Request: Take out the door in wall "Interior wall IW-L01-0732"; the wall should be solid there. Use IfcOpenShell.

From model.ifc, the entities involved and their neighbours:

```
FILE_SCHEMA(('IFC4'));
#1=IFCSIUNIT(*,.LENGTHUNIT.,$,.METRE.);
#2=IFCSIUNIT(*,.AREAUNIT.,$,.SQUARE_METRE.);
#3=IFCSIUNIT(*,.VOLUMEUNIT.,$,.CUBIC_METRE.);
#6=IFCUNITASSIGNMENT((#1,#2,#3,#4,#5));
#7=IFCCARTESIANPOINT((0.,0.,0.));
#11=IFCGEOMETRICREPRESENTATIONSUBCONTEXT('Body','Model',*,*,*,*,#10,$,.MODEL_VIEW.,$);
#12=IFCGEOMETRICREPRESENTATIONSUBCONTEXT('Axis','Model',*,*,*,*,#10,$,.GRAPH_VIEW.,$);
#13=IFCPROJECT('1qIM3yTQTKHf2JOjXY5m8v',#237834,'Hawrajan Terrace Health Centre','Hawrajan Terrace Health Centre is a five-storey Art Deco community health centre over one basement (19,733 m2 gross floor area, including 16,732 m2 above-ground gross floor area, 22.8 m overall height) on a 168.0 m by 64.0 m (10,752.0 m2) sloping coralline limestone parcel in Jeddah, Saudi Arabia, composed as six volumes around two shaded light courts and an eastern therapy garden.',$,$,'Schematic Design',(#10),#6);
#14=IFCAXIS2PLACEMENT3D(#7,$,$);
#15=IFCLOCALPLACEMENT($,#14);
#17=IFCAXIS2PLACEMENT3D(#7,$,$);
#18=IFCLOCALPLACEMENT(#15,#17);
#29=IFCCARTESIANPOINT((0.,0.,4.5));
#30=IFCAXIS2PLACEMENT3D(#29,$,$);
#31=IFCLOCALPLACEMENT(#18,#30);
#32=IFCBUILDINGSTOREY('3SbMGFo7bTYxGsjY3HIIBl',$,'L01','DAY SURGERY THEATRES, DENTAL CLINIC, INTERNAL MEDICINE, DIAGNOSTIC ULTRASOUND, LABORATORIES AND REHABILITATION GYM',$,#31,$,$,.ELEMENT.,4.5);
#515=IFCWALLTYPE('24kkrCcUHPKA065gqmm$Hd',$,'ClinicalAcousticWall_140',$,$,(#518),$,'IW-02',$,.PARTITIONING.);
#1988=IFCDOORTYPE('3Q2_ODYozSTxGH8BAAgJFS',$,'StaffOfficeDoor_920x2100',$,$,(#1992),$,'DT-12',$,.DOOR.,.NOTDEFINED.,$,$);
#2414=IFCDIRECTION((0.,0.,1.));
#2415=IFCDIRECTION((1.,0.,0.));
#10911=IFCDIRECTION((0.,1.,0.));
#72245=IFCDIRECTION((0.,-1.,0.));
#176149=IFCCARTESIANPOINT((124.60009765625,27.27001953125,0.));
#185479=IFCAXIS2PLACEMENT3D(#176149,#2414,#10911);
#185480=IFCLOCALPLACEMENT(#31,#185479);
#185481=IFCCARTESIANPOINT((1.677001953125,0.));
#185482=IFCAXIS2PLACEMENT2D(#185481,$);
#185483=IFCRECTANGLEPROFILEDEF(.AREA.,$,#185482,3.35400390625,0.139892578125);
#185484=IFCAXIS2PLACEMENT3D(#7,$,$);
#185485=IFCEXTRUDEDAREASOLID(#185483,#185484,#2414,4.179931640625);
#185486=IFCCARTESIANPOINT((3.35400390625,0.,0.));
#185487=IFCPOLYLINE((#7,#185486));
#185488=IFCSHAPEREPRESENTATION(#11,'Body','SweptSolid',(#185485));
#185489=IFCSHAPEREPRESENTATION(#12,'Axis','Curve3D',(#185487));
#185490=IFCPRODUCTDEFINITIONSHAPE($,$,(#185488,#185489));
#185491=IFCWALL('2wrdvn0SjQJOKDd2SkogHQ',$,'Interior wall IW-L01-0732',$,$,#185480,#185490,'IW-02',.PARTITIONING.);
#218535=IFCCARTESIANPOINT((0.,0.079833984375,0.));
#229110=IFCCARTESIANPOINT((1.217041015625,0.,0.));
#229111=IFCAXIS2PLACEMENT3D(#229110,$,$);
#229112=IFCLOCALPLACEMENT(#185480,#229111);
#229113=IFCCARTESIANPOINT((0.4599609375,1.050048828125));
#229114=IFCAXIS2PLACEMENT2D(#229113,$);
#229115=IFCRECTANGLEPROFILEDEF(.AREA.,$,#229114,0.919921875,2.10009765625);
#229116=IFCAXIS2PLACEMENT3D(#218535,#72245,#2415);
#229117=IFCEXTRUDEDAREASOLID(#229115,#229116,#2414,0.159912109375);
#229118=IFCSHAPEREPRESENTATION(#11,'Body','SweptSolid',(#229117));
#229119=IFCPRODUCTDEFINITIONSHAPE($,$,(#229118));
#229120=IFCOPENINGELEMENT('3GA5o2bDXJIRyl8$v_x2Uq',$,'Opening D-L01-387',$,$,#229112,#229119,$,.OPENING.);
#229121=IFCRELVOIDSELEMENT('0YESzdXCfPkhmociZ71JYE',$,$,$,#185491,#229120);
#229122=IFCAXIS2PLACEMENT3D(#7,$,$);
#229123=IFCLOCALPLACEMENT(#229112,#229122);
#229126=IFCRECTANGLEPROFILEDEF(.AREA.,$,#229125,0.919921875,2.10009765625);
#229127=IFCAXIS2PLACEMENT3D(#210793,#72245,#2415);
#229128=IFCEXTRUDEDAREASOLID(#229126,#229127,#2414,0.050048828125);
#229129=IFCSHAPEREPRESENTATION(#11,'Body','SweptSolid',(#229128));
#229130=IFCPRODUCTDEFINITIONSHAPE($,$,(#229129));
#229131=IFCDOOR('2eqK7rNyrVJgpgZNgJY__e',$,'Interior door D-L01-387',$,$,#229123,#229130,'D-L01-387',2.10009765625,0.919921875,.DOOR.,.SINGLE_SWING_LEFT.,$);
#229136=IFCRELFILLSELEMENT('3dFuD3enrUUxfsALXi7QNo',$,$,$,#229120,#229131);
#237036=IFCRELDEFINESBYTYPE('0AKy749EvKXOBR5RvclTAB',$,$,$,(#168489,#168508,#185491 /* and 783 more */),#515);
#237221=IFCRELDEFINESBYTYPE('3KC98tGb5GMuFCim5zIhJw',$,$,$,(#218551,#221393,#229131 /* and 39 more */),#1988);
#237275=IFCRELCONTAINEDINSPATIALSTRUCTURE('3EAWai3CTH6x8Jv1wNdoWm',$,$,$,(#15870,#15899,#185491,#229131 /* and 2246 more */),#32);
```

```python
import ifcopenshell
import ifcopenshell.api.feature
import ifcopenshell.api.root
import ifcopenshell.geom
import ifcopenshell.util.shape

model = ifcopenshell.open("model.ifc")
settings = ifcopenshell.geom.settings()


def volume(element):
    """Net volume in cubic metres, openings subtracted."""
    shape = ifcopenshell.geom.create_shape(settings, element)
    return ifcopenshell.util.shape.get_volume(shape.geometry)


door = model.by_id(229131)
opening = door.FillsVoids[0].RelatingOpeningElement
wall = opening.VoidsElements[0].RelatingBuildingElement
before = volume(wall)

ifcopenshell.api.root.remove_product(model, product=door)
ifcopenshell.api.feature.remove_feature(model, feature=opening)

after = volume(wall)

print(f"wall volume {before:.3f} -> {after:.3f} m3")

model.write("model_rev.ifc")
```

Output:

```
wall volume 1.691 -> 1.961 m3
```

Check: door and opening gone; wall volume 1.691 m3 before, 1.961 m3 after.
